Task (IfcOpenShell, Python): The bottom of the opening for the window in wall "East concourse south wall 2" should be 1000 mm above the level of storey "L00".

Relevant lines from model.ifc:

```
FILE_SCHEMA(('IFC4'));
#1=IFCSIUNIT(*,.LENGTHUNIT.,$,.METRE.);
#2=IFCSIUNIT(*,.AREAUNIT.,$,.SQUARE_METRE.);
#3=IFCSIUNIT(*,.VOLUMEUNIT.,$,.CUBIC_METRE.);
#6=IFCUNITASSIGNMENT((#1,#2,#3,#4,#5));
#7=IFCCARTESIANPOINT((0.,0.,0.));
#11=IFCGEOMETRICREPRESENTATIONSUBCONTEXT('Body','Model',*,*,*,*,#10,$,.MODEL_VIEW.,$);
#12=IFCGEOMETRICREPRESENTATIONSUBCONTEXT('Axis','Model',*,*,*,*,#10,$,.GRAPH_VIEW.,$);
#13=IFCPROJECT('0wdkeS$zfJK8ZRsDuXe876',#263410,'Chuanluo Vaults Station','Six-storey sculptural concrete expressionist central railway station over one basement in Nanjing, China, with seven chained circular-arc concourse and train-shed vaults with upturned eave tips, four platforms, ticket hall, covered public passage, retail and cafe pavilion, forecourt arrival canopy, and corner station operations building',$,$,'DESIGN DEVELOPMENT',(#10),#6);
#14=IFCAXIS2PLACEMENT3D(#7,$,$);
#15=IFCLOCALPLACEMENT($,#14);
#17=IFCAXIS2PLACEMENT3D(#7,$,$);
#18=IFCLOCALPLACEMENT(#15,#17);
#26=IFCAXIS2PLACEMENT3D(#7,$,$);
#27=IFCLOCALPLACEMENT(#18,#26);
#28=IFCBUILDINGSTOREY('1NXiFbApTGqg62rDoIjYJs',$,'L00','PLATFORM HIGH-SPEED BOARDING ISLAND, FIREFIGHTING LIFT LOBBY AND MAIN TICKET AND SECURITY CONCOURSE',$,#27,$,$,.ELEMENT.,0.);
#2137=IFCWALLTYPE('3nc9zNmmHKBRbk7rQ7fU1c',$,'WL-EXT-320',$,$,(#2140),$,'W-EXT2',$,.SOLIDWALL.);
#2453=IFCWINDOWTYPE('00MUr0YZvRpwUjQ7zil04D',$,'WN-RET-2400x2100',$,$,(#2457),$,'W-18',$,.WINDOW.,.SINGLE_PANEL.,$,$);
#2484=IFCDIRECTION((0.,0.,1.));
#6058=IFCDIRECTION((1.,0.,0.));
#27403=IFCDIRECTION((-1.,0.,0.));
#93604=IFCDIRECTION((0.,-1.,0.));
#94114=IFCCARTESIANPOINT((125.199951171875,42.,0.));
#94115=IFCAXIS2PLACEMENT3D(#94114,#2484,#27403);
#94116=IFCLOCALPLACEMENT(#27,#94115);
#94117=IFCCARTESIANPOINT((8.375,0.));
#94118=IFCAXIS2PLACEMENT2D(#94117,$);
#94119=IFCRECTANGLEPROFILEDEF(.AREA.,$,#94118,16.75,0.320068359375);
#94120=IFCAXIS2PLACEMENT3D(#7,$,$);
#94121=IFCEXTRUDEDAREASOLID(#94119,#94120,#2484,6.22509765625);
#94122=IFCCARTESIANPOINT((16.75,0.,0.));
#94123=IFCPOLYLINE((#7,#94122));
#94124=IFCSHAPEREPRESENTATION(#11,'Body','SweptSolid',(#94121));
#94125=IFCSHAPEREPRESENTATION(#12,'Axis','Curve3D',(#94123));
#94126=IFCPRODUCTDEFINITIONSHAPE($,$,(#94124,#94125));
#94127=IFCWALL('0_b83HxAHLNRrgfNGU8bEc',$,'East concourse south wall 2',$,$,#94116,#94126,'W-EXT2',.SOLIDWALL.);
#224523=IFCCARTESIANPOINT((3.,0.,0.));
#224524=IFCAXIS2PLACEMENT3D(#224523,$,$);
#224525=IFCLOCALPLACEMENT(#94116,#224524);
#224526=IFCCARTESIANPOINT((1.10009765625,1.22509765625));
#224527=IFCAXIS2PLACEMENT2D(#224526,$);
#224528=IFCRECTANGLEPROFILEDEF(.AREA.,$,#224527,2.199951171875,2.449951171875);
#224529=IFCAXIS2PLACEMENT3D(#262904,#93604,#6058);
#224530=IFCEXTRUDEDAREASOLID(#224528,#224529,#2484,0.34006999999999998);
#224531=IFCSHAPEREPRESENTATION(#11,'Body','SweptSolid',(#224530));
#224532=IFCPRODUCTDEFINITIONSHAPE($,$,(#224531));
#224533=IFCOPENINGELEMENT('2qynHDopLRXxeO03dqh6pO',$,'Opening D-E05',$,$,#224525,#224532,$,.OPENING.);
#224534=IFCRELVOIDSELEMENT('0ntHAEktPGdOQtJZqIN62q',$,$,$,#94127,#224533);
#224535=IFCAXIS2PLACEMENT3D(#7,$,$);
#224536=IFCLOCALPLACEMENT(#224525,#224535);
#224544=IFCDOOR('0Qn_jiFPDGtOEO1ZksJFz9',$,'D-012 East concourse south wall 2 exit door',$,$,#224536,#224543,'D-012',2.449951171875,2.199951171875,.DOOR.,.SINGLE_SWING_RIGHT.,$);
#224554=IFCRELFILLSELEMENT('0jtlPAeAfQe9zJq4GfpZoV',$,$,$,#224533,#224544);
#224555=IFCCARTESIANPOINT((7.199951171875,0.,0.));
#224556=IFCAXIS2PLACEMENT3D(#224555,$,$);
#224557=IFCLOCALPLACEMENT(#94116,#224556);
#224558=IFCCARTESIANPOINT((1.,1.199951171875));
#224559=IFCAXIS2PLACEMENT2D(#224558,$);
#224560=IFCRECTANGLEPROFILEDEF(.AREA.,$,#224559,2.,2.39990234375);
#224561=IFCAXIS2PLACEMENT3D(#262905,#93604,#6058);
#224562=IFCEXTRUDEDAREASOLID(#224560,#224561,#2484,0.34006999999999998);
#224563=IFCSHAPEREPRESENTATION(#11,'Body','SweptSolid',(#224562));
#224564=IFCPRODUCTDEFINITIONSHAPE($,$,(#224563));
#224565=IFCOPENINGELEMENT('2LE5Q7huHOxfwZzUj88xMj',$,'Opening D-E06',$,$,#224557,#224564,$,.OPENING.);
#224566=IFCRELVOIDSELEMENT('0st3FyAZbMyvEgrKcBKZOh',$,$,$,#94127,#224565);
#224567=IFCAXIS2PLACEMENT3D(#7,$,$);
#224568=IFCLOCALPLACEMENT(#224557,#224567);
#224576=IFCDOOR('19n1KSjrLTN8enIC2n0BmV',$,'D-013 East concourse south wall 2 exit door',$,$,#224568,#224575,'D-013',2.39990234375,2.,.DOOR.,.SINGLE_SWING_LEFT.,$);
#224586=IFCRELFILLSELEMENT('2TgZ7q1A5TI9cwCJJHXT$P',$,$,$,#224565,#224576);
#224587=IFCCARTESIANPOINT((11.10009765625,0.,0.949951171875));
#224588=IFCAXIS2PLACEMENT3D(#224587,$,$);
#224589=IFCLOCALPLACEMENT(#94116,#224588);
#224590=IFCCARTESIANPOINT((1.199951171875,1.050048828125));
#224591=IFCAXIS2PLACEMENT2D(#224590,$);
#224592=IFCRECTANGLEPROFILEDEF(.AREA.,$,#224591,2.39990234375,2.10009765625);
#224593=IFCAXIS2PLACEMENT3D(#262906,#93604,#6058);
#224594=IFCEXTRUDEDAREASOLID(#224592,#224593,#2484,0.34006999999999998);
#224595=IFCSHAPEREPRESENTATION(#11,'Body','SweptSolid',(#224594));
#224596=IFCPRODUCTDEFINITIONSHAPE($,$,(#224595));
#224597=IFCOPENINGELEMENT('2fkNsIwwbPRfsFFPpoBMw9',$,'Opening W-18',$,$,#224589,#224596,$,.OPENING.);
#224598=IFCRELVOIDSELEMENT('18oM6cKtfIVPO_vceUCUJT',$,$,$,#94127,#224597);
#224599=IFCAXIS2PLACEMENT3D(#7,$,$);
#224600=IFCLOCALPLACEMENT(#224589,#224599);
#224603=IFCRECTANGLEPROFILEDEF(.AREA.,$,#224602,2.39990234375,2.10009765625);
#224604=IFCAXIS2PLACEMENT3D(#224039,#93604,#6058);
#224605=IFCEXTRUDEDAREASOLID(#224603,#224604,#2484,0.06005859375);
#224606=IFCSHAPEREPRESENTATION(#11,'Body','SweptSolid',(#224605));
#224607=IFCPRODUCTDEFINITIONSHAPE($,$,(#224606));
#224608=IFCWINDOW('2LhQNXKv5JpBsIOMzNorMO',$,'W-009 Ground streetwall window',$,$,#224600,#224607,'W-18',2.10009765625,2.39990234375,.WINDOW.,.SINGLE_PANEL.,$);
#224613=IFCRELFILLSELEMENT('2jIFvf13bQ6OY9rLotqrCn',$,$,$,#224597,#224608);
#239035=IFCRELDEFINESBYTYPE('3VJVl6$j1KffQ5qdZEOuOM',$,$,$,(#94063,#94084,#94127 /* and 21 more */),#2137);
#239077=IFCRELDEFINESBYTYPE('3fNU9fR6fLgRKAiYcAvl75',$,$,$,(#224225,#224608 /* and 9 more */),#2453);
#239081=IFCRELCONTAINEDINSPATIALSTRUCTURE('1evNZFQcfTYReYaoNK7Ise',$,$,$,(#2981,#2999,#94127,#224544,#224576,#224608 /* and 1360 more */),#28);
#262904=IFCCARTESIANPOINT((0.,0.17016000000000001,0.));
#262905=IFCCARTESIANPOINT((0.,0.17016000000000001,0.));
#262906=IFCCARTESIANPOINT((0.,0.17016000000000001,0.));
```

```python
import numpy as np
import ifcopenshell
import ifcopenshell.api.geometry
import ifcopenshell.geom
import ifcopenshell.util.element
import ifcopenshell.util.placement
import ifcopenshell.util.shape
import ifcopenshell.util.unit

model = ifcopenshell.open("model.ifc")
unit_scale = ifcopenshell.util.unit.calculate_unit_scale(model)

window = model.by_id(224608)
opening = window.FillsVoids[0].RelatingOpeningElement
storey = ifcopenshell.util.element.get_container(window, ifc_class="IfcBuildingStorey")
level = ifcopenshell.util.placement.get_local_placement(storey.ObjectPlacement)[2, 3]

# The opening's origin need not be at the sill, so measure its lowest point.
shape = ifcopenshell.geom.create_shape(ifcopenshell.geom.settings(), opening)
bottom = ifcopenshell.util.shape.get_shape_bottom_elevation(shape, shape.geometry) / unit_scale
dz = level + 1.0 - bottom

shift = np.array([0.0, 0.0, dz])
# The window is placed relative to its opening, so it follows when the opening moves.
matrix = ifcopenshell.util.placement.get_local_placement(opening.ObjectPlacement)
matrix[:3, 3] += shift
ifcopenshell.api.geometry.edit_object_placement(
    model, product=opening, matrix=matrix, is_si=False, should_transform_children=True
)

print(f"moved by {dz * unit_scale:+.3f} m")

model.write("model_v2.ifc")
```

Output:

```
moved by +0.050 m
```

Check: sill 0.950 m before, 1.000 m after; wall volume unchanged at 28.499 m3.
